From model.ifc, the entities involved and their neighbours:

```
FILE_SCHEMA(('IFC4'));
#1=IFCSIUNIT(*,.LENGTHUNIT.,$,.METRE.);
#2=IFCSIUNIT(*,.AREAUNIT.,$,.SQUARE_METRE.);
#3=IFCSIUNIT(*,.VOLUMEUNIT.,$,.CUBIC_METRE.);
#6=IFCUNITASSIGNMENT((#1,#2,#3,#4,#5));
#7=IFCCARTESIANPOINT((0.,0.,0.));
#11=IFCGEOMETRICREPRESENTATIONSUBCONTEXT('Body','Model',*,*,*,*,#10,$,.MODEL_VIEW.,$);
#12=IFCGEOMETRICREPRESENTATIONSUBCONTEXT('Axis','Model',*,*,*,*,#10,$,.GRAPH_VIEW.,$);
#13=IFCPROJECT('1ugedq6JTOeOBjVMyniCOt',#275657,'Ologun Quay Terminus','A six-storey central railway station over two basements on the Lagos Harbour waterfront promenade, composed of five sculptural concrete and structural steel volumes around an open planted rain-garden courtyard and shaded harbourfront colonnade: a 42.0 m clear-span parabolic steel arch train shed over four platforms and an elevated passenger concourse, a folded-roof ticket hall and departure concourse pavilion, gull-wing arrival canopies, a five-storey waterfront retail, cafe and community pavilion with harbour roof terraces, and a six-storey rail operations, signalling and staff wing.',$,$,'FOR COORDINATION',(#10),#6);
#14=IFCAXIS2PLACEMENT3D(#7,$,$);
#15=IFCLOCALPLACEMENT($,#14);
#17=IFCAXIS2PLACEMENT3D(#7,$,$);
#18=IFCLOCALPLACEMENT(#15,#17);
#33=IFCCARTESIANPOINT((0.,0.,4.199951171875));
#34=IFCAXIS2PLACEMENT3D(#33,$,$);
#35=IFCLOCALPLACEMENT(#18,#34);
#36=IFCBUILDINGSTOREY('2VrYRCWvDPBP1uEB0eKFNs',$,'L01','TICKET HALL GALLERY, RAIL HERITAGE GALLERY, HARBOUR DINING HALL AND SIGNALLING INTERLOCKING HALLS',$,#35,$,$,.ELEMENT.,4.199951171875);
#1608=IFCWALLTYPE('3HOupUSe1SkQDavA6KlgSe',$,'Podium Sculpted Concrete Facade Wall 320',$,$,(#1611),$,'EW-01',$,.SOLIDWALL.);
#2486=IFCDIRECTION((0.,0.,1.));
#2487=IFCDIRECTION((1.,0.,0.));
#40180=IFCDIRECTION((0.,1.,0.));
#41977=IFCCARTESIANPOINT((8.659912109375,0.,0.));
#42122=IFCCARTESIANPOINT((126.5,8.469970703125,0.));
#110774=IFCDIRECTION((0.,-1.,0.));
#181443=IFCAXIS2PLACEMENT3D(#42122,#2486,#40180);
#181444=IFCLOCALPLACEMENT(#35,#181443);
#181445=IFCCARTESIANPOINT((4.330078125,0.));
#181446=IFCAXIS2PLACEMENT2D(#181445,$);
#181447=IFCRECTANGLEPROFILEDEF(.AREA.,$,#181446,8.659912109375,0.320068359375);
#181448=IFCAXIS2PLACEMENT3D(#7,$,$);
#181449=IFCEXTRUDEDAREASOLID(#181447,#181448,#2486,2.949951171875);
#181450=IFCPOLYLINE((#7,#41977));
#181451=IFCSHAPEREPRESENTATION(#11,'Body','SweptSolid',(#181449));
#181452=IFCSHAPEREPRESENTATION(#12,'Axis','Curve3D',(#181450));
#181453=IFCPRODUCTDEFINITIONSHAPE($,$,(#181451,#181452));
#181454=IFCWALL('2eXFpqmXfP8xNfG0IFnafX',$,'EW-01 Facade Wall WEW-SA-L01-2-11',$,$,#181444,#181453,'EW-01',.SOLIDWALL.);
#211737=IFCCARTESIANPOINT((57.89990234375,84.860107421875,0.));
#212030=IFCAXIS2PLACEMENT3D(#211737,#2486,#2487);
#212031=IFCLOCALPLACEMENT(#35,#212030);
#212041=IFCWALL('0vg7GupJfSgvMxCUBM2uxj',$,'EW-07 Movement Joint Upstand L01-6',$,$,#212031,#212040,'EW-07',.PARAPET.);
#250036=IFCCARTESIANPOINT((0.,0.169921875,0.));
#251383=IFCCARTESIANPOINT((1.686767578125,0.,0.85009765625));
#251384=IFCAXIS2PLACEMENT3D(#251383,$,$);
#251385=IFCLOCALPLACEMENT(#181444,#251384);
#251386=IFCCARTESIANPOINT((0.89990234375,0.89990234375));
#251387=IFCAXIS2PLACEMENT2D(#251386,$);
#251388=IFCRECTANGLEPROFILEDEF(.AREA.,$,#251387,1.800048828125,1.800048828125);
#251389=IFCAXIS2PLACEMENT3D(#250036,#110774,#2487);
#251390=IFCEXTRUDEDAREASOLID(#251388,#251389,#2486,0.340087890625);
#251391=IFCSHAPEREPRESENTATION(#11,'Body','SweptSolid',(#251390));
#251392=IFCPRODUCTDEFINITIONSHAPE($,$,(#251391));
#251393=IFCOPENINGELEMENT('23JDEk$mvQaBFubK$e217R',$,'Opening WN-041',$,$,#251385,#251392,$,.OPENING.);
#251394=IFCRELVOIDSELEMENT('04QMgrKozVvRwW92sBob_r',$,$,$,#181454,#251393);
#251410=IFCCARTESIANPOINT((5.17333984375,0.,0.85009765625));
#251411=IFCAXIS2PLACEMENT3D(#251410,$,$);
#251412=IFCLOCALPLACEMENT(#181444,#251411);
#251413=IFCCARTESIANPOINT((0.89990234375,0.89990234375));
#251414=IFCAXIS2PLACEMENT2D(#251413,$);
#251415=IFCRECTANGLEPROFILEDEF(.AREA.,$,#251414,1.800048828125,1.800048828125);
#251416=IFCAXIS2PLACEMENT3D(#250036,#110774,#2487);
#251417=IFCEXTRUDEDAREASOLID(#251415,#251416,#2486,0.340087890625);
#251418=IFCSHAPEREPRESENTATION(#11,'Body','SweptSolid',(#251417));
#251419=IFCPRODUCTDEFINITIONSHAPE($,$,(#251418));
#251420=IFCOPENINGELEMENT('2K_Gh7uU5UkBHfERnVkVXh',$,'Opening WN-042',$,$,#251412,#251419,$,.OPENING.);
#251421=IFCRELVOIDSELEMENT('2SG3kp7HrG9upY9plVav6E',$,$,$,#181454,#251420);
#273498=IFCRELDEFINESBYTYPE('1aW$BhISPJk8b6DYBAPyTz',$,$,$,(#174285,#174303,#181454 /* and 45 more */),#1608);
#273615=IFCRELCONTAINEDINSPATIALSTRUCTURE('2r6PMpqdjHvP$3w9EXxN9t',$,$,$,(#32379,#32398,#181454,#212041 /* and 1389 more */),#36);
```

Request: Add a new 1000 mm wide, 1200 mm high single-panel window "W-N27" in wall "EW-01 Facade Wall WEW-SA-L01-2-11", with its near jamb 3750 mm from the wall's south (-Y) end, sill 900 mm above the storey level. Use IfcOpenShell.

```python
import numpy as np
import ifcopenshell
import ifcopenshell.api.feature
import ifcopenshell.api.geometry
import ifcopenshell.api.root
import ifcopenshell.api.spatial
import ifcopenshell.geom
import ifcopenshell.util.element
import ifcopenshell.util.placement
import ifcopenshell.util.representation
import ifcopenshell.util.shape
import ifcopenshell.util.unit

model = ifcopenshell.open("model.ifc")
unit_scale = ifcopenshell.util.unit.calculate_unit_scale(model)
settings = ifcopenshell.geom.settings()


def volume(element):
    """Net volume in cubic metres, openings subtracted."""
    shape = ifcopenshell.geom.create_shape(settings, element)
    return ifcopenshell.util.shape.get_volume(shape.geometry)


wall = model.by_guid("2eXFpqmXfP8xNfG0IFnafX")
storey = ifcopenshell.util.element.get_container(wall, ifc_class="IfcBuildingStorey")
context = ifcopenshell.util.representation.get_context(model, "Model", "Body", "MODEL_VIEW")
before = volume(wall)

width, height, from_end, sill = 1, 1.2, 3.75, 0.9  # metres

# The wall runs along its own X axis, and the end named is its -X end.
wall_shape = ifcopenshell.geom.create_shape(settings, wall)
x, y, z = ifcopenshell.util.shape.get_vertices(wall_shape.geometry).T
start = x.min() + from_end
face, thickness = float(y.min()), float(y.max() - y.min())
wall_matrix = ifcopenshell.util.placement.get_local_placement(wall.ObjectPlacement)
level = ifcopenshell.util.placement.get_local_placement(storey.ObjectPlacement)[2, 3]


def in_wall(x, y):
    """Placement at x, y metres in the wall's axes, at sill height."""
    matrix = wall_matrix.copy()
    matrix[:, 3] = wall_matrix @ np.array([x / unit_scale, y / unit_scale, 0.0, 1.0])
    matrix[2, 3] = level + sill / unit_scale
    return matrix


# Opening: a box that overshoots both wall faces by 50 mm.
opening = ifcopenshell.api.root.create_entity(model, ifc_class="IfcOpeningElement", predefined_type="OPENING")
box = ifcopenshell.api.geometry.add_wall_representation(
    model, context=context, length=width, height=height, thickness=thickness + 0.1
)
ifcopenshell.api.geometry.assign_representation(model, product=opening, representation=box)
ifcopenshell.api.geometry.edit_object_placement(model, product=opening, matrix=in_wall(start, face - 0.05), is_si=False)
ifcopenshell.api.feature.add_feature(model, feature=opening, element=wall)

window = ifcopenshell.api.root.create_entity(model, ifc_class="IfcWindow", name="W-N27", predefined_type="WINDOW")
window.OverallWidth, window.OverallHeight = width / unit_scale, height / unit_scale
window.PartitioningType = "SINGLE_PANEL"
body = ifcopenshell.api.geometry.add_window_representation(
    model,
    context=context,
    overall_width=window.OverallWidth,
    overall_height=window.OverallHeight,
    partition_type="SINGLE_PANEL",
)
ifcopenshell.api.geometry.assign_representation(model, product=window, representation=body)
ifcopenshell.api.spatial.assign_container(model, products=[window], relating_structure=storey)
ifcopenshell.api.feature.add_filling(model, opening=opening, element=window)

# Centre the window in the wall's thickness.
ifcopenshell.api.geometry.edit_object_placement(model, product=window, matrix=in_wall(start, face), is_si=False)
window_shape = ifcopenshell.geom.create_shape(settings, window)
depth = ifcopenshell.util.shape.get_vertices(window_shape.geometry)[:, 1]
offset = face + thickness / 2 - (depth.min() + depth.max()) / 2
ifcopenshell.api.geometry.edit_object_placement(model, product=window, matrix=in_wall(start, offset), is_si=False)

after = volume(wall)

print(f"wall volume {before:.3f} -> {after:.3f} m3")

model.write("model-out.ifc")
```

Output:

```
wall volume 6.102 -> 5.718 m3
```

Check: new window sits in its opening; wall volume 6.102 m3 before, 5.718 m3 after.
